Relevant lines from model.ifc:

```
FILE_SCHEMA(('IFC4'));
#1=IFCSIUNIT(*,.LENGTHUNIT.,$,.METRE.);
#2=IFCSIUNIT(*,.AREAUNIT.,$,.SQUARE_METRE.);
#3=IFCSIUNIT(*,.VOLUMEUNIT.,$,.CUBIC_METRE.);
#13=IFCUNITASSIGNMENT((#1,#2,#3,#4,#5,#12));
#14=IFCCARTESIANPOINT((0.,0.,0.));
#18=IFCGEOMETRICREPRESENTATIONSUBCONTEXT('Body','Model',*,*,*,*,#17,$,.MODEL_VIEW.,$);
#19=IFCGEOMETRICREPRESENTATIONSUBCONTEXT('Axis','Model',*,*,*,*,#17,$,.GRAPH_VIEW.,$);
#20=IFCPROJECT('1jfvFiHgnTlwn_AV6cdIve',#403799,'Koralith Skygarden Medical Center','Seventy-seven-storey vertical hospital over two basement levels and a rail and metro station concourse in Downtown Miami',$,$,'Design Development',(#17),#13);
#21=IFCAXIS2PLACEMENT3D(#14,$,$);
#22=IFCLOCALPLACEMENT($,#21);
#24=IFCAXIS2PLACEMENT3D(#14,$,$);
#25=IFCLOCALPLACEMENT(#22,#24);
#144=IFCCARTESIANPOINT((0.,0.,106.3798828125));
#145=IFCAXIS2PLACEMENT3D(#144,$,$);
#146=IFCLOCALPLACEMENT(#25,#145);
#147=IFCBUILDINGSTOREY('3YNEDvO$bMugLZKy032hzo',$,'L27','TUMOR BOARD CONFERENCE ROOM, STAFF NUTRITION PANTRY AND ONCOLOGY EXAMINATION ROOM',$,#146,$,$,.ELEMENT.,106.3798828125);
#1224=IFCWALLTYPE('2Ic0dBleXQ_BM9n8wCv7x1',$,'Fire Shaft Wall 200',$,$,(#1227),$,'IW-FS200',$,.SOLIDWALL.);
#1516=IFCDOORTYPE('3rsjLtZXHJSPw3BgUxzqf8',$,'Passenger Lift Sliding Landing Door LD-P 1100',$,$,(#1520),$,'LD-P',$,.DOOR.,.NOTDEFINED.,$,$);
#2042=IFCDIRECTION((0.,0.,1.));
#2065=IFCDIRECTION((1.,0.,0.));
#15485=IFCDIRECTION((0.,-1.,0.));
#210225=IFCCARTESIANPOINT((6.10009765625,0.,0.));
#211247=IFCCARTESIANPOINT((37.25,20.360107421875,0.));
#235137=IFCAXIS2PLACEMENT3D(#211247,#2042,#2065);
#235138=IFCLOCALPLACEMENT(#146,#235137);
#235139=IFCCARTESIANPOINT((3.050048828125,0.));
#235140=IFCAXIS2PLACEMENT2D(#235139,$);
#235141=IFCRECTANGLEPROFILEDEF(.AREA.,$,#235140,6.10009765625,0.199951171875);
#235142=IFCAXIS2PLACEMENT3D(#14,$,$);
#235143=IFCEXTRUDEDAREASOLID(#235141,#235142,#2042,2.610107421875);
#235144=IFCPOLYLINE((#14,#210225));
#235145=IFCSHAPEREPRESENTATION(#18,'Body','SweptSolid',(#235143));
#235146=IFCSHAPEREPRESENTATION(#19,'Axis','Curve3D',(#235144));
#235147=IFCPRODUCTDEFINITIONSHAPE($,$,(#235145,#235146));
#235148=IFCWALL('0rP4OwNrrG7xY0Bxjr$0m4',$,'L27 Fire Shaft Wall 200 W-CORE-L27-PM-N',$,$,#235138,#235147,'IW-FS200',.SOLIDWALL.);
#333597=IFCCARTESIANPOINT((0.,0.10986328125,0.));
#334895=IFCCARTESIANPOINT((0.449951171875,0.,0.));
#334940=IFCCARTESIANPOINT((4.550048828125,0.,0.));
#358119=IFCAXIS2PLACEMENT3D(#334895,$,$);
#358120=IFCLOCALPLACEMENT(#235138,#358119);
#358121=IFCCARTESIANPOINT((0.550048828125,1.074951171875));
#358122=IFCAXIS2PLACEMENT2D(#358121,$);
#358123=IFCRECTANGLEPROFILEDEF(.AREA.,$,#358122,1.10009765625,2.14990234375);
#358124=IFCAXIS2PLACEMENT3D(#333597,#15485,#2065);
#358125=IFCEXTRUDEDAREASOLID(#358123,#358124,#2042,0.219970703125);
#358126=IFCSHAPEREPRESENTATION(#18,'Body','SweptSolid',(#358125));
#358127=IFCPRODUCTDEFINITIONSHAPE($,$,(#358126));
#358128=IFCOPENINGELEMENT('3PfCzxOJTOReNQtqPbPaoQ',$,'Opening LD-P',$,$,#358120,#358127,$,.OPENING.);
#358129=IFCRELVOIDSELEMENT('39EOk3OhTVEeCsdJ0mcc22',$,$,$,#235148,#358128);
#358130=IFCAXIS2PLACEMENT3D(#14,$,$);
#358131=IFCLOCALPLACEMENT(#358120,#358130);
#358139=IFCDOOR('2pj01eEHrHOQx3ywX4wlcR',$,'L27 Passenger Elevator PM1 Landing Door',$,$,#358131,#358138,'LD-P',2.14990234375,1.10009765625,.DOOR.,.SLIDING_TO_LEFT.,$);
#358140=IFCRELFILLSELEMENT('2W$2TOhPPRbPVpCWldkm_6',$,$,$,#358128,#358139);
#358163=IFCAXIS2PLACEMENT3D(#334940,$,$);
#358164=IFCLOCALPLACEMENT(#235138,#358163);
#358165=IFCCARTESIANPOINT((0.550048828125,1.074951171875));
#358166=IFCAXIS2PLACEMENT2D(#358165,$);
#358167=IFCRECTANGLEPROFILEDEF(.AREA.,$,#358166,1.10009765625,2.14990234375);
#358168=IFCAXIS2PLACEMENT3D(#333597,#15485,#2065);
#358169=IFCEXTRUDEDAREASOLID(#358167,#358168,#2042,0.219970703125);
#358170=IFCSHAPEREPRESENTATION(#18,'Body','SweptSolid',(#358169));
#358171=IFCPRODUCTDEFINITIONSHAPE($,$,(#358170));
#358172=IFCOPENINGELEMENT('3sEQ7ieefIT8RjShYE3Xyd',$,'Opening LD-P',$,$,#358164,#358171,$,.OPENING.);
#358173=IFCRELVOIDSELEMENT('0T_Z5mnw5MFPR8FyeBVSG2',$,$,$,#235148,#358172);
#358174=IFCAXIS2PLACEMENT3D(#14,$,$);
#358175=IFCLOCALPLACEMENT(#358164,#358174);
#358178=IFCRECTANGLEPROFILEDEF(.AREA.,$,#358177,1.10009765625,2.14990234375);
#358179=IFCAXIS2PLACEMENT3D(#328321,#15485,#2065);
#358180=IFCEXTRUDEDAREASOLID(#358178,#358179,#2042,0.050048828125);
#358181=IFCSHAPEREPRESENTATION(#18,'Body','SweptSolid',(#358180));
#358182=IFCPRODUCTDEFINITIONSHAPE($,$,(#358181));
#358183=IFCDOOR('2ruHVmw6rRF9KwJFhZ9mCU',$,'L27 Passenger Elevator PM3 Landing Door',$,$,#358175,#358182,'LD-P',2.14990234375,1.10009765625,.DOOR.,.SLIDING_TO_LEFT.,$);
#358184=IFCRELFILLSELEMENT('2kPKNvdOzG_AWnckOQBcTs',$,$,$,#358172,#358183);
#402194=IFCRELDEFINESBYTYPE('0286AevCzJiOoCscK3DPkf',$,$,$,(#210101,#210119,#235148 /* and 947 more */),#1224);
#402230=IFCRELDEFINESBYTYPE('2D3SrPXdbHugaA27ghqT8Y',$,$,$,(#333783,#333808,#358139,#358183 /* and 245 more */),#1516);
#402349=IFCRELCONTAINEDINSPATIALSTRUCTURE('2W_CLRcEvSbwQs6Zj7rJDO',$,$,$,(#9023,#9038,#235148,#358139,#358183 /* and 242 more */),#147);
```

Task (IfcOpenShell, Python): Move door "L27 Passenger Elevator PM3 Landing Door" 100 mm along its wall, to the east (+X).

```python
import ifcopenshell
import ifcopenshell.api.geometry
import ifcopenshell.util.placement
import ifcopenshell.util.unit

model = ifcopenshell.open("model.ifc")
unit_scale = ifcopenshell.util.unit.calculate_unit_scale(model)

door = model.by_guid("2ruHVmw6rRF9KwJFhZ9mCU")
opening = door.FillsVoids[0].RelatingOpeningElement
wall = opening.VoidsElements[0].RelatingBuildingElement

wall_matrix = ifcopenshell.util.placement.get_local_placement(wall.ObjectPlacement)
shift = wall_matrix[:3, 0] * 0.1 / unit_scale
before = ifcopenshell.util.placement.get_local_placement(door.ObjectPlacement)[:3, 3].copy()

# The door is placed relative to its opening, so it follows when the opening moves.
matrix = ifcopenshell.util.placement.get_local_placement(opening.ObjectPlacement)
matrix[:3, 3] += shift
ifcopenshell.api.geometry.edit_object_placement(
    model, product=opening, matrix=matrix, is_si=False, should_transform_children=True
)

after = ifcopenshell.util.placement.get_local_placement(door.ObjectPlacement)[:3, 3]
print("door moved by", (after - before).round(3) + 0.0)

model.write("model_v2.ifc")
```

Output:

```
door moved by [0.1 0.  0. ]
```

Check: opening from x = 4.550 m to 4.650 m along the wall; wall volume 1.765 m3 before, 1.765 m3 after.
